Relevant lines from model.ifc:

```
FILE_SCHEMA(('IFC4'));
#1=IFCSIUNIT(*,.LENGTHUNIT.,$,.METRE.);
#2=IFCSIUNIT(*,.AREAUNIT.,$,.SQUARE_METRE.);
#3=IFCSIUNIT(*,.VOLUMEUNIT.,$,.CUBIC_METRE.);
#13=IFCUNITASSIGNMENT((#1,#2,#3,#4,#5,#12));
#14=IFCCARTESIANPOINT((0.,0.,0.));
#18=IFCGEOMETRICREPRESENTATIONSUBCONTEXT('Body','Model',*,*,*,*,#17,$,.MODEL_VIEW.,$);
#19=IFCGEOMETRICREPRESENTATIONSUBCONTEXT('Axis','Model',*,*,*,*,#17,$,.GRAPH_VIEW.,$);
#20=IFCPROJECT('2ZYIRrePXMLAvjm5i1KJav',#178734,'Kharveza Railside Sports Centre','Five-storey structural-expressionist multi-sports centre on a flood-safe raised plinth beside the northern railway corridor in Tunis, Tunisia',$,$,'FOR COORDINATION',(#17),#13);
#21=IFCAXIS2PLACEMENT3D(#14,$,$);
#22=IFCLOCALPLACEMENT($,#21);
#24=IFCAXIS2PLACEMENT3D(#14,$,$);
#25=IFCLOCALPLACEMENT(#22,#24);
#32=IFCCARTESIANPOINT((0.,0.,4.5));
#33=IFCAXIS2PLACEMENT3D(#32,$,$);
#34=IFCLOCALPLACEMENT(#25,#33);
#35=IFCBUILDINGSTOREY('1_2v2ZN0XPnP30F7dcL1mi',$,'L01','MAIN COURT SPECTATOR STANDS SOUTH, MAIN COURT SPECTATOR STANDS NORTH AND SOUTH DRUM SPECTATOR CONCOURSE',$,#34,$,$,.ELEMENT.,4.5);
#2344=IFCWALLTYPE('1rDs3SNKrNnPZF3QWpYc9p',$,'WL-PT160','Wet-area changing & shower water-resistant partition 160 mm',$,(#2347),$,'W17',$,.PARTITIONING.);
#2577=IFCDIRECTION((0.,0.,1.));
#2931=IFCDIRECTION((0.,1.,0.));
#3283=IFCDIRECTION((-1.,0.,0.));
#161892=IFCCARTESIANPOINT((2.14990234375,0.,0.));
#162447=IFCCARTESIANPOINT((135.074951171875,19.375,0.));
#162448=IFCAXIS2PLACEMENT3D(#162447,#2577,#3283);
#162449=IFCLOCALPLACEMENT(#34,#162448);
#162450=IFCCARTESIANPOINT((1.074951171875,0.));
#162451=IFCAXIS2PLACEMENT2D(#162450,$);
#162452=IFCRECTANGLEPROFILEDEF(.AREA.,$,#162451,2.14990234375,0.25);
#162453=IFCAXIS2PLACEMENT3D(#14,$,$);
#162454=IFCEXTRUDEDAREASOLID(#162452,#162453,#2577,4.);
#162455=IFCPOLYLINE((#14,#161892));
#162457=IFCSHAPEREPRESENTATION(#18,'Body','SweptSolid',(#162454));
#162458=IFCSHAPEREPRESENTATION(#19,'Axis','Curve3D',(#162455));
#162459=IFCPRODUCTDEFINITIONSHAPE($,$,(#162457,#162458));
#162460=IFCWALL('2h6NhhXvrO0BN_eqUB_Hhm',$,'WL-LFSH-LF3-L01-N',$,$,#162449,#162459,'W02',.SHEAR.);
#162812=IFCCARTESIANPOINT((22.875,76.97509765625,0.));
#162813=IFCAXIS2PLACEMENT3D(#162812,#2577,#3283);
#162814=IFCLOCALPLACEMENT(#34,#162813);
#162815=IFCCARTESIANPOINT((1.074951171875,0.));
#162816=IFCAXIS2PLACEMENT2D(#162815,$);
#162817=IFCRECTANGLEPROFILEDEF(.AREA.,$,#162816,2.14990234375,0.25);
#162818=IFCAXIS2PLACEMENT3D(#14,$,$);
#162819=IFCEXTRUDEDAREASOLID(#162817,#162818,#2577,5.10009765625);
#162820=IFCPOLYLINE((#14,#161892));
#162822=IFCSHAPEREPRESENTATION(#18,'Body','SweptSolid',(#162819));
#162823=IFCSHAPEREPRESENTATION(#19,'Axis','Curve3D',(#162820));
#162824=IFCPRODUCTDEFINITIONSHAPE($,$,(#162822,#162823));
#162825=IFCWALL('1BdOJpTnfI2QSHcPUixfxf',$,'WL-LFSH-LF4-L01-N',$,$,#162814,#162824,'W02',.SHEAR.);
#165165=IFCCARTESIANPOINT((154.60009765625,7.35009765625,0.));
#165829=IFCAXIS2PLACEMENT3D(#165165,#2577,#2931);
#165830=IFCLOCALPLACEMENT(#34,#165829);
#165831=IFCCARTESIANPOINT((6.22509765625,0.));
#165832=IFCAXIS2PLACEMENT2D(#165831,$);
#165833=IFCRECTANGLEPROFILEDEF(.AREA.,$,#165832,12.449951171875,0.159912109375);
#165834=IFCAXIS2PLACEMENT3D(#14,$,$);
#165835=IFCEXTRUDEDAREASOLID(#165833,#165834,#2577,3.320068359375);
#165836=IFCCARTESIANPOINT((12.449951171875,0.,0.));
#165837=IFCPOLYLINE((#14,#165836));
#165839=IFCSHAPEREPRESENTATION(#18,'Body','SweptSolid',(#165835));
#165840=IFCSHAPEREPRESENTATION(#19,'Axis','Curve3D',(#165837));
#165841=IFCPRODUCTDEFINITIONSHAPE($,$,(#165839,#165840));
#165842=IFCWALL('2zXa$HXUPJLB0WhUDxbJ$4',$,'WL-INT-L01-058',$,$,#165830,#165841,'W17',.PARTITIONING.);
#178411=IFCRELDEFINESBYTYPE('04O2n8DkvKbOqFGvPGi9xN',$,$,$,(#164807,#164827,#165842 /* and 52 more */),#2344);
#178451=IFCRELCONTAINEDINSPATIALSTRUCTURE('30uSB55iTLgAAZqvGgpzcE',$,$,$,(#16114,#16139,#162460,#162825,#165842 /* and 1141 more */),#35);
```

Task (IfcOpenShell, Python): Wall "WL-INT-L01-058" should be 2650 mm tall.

```python
import ifcopenshell
import ifcopenshell.geom
import ifcopenshell.util.representation
import ifcopenshell.util.shape
import ifcopenshell.util.unit

model = ifcopenshell.open("model.ifc")
unit_scale = ifcopenshell.util.unit.calculate_unit_scale(model)
settings = ifcopenshell.geom.settings()


def volume(element):
    """Net volume in cubic metres, openings subtracted."""
    shape = ifcopenshell.geom.create_shape(settings, element)
    return ifcopenshell.util.shape.get_volume(shape.geometry)


wall = model.by_guid("2zXa$HXUPJLB0WhUDxbJ$4")
before = volume(wall)

body = ifcopenshell.util.representation.get_representation(wall, "Model", "Body")
solid = body.Items[0]
old_height = solid.Depth
solid.Depth = 2.65 / unit_scale
after = volume(wall)

print(f"height {old_height:g} -> {solid.Depth:g}, volume {before:.3f} -> {after:.3f} m3")

model.write("model_v2.ifc")
```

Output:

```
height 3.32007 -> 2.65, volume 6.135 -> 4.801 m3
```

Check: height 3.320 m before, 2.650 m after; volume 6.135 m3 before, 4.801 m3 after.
